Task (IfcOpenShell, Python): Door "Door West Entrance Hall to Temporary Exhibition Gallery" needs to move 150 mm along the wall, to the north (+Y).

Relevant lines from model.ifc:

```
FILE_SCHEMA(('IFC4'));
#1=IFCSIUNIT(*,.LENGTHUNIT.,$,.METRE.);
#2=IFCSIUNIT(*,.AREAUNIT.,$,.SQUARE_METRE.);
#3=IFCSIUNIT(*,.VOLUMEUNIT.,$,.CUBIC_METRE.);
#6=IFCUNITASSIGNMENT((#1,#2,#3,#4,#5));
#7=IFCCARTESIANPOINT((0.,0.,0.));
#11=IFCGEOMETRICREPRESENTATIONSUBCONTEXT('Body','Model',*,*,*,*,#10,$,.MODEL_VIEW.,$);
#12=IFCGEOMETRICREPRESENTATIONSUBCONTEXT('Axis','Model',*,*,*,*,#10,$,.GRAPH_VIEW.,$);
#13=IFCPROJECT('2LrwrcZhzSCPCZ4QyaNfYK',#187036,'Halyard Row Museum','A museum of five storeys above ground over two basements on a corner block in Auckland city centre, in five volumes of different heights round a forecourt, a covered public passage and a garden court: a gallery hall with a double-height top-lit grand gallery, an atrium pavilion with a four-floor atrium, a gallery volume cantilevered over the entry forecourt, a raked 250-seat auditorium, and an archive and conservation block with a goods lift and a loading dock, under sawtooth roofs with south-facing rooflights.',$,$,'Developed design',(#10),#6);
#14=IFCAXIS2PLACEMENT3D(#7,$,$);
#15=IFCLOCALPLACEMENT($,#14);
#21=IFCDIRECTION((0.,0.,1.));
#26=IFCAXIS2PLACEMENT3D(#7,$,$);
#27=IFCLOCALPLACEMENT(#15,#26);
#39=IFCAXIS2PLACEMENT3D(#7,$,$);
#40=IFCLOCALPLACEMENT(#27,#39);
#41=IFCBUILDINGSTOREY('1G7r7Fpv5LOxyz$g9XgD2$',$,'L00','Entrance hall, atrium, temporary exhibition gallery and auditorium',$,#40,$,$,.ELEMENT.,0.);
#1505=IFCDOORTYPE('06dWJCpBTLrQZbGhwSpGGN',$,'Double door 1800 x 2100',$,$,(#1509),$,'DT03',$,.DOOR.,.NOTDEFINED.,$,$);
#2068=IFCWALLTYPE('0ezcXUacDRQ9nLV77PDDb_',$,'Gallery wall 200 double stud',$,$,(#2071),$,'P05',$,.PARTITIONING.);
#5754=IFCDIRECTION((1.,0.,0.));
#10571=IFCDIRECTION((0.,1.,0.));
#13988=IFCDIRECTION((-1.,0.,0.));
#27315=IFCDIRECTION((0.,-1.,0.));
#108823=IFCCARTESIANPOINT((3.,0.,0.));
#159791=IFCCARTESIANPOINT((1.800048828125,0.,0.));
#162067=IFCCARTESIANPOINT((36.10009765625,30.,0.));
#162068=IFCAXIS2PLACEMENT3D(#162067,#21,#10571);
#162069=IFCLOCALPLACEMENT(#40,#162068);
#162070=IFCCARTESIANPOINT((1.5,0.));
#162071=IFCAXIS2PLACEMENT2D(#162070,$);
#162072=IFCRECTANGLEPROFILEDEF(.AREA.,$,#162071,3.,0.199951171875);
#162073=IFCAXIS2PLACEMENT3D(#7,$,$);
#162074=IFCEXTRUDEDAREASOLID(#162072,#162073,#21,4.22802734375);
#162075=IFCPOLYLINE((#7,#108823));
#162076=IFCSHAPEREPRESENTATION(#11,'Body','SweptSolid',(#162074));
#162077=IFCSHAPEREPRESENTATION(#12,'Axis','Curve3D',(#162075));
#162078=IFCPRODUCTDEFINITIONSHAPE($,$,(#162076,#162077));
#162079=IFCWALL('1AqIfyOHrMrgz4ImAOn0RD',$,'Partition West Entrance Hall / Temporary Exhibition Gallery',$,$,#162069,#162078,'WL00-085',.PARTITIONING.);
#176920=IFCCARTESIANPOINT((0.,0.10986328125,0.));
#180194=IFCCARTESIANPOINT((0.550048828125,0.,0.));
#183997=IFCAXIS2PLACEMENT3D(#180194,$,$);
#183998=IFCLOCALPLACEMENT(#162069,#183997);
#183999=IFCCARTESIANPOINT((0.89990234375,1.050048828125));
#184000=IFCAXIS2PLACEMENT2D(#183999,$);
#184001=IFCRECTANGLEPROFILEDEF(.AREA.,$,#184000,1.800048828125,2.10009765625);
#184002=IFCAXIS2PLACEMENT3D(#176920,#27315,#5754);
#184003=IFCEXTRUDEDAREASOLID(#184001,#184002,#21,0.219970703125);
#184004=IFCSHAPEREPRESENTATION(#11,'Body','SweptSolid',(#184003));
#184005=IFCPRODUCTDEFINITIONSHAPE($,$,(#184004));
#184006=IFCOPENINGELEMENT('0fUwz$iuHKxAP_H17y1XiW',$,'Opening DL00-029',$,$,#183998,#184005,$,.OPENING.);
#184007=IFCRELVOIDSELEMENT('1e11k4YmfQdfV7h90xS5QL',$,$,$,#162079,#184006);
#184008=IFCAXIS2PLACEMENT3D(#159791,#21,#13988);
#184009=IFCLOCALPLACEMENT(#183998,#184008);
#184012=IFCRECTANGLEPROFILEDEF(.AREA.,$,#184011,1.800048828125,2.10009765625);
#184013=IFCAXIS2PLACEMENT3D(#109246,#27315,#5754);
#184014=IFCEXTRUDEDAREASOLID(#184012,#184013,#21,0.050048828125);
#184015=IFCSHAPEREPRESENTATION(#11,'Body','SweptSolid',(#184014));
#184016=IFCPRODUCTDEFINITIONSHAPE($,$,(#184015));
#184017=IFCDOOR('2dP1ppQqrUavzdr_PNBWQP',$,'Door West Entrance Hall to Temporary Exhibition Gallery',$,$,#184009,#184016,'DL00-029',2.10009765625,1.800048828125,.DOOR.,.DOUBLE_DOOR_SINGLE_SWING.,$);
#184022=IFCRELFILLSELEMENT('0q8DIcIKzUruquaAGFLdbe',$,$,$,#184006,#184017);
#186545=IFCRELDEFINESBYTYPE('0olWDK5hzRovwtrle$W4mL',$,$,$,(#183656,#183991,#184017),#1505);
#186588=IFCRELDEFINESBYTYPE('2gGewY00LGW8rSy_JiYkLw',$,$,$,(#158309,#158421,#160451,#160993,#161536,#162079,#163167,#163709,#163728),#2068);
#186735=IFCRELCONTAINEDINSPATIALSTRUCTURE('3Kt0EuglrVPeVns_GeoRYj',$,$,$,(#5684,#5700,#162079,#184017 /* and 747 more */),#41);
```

```python
import ifcopenshell
import ifcopenshell.api.geometry
import ifcopenshell.util.placement
import ifcopenshell.util.unit

model = ifcopenshell.open("model.ifc")
unit_scale = ifcopenshell.util.unit.calculate_unit_scale(model)

door = model.by_id(184017)
opening = door.FillsVoids[0].RelatingOpeningElement
wall = opening.VoidsElements[0].RelatingBuildingElement

wall_matrix = ifcopenshell.util.placement.get_local_placement(wall.ObjectPlacement)
shift = wall_matrix[:3, 0] * 0.15 / unit_scale
before = ifcopenshell.util.placement.get_local_placement(door.ObjectPlacement)[:3, 3].copy()

# The door is placed relative to its opening, so it follows when the opening moves.
matrix = ifcopenshell.util.placement.get_local_placement(opening.ObjectPlacement)
matrix[:3, 3] += shift
ifcopenshell.api.geometry.edit_object_placement(
    model, product=opening, matrix=matrix, is_si=False, should_transform_children=True
)

after = ifcopenshell.util.placement.get_local_placement(door.ObjectPlacement)[:3, 3]
print("door moved by", (after - before).round(3) + 0.0)

model.write("model-out.ifc")
```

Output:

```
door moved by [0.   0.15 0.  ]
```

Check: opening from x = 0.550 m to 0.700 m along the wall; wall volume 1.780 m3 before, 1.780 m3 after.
